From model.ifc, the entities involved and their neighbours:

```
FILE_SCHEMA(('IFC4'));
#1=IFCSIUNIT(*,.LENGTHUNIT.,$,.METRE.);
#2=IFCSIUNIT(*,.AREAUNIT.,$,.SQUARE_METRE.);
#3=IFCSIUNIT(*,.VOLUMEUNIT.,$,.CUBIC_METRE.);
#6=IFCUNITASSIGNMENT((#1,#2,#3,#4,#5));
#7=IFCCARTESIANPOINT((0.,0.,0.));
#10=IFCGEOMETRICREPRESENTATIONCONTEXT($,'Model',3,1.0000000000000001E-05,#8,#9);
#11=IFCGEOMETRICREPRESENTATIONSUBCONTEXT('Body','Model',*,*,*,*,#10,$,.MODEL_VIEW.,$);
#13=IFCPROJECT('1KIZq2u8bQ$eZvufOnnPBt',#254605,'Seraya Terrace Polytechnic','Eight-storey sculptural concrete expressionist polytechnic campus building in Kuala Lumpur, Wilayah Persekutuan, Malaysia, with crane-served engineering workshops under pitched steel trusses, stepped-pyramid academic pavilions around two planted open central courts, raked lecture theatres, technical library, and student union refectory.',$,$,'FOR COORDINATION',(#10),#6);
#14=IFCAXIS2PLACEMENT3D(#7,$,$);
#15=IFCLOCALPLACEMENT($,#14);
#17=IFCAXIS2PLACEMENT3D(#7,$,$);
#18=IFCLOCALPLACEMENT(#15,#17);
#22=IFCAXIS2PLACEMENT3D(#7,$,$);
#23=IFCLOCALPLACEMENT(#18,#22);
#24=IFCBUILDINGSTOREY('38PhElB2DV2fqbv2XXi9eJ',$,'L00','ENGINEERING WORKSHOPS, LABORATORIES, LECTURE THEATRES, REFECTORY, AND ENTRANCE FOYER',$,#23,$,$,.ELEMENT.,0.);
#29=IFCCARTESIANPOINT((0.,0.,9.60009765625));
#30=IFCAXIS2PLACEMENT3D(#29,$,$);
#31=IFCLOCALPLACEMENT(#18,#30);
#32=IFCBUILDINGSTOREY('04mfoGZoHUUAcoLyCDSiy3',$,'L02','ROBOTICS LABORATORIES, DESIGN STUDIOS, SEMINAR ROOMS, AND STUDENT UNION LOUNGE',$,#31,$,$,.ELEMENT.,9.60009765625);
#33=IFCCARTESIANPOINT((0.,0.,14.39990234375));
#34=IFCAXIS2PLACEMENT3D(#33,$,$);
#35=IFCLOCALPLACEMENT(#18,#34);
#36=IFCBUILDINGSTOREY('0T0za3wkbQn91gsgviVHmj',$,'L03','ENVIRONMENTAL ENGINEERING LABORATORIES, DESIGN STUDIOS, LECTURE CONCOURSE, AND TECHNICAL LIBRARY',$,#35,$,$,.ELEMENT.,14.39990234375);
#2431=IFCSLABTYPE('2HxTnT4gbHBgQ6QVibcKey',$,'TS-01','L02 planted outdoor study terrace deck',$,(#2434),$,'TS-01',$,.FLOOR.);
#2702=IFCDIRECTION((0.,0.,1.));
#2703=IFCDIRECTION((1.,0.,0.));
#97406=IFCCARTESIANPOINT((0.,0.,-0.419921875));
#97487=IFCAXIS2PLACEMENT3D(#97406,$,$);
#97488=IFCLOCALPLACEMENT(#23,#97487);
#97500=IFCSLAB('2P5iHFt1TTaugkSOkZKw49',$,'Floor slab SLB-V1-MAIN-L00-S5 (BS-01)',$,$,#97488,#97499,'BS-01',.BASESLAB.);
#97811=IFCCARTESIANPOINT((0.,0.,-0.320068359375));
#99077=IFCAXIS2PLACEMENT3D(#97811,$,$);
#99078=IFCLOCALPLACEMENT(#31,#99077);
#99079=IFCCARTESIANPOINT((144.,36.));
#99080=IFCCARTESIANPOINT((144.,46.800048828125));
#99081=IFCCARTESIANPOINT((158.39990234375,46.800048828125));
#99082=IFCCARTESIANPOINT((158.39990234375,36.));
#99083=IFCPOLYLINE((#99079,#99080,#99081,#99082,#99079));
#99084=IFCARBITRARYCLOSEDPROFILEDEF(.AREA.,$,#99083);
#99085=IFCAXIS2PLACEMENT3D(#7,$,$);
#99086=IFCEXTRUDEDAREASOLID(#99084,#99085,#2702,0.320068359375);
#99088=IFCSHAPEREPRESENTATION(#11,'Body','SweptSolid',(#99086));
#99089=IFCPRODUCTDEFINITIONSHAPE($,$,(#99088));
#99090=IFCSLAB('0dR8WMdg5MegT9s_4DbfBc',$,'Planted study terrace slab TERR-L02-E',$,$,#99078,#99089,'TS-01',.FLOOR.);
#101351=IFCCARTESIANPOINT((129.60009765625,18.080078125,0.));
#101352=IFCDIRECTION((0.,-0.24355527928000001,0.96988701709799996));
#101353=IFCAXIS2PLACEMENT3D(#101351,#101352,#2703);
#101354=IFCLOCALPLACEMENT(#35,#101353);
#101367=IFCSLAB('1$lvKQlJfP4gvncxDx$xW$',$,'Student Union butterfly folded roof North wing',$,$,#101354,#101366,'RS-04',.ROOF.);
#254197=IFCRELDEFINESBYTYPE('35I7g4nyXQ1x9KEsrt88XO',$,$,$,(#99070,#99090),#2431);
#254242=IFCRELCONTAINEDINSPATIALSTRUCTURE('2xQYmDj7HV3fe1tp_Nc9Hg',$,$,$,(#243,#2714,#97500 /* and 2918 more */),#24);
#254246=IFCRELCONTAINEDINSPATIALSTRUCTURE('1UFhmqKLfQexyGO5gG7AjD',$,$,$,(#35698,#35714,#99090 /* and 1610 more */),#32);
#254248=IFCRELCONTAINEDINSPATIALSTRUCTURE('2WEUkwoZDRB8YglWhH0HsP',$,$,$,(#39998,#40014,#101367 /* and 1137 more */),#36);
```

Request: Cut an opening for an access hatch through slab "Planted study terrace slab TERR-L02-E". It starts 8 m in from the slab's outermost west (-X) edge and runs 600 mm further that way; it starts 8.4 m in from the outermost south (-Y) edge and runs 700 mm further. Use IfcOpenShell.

```python
import numpy as np
import ifcopenshell
import ifcopenshell.api.feature
import ifcopenshell.api.geometry
import ifcopenshell.api.root
import ifcopenshell.geom
import ifcopenshell.util.placement
import ifcopenshell.util.representation
import ifcopenshell.util.shape
import ifcopenshell.util.unit

model = ifcopenshell.open("model.ifc")
unit_scale = ifcopenshell.util.unit.calculate_unit_scale(model)
settings = ifcopenshell.geom.settings()


def volume(element):
    """Net volume in cubic metres, openings subtracted."""
    shape = ifcopenshell.geom.create_shape(settings, element)
    return ifcopenshell.util.shape.get_volume(shape.geometry)


slab = model.by_guid("0dR8WMdg5MegT9s_4DbfBc")
before = volume(slab)

# Extent in the slab's own axes, in metres. The edges named are its -X and -Y sides.
slab_shape = ifcopenshell.geom.create_shape(settings, slab)
vertices = ifcopenshell.util.shape.get_vertices(slab_shape.geometry)
x_min, y_min, bottom = vertices.min(axis=0)
top = vertices[:, 2].max()

opening = ifcopenshell.api.root.create_entity(model, ifc_class="IfcOpeningElement", name="Access hatch opening", predefined_type="OPENING")
context = ifcopenshell.util.representation.get_context(model, "Model", "Body", "MODEL_VIEW")
width, depth = 0.6, 0.7
outline = [(0.0, 0.0), (width, 0.0), (width, depth), (0.0, depth), (0.0, 0.0)]
# Overshoot both faces by 50 mm so the cut is clean.
shape = ifcopenshell.api.geometry.add_slab_representation(
    model, context=context, depth=top - bottom + 0.1, polyline=outline
)
ifcopenshell.api.geometry.assign_representation(model, product=opening, representation=shape)

matrix = ifcopenshell.util.placement.get_local_placement(slab.ObjectPlacement)
matrix[:, 3] = matrix @ np.append(np.array([x_min + 8, y_min + 8.4, bottom - 0.05]) / unit_scale, 1.0)
ifcopenshell.api.geometry.edit_object_placement(model, product=opening, matrix=matrix, is_si=False)
ifcopenshell.api.feature.add_feature(model, feature=opening, element=slab)

after = volume(slab)

print(f"slab volume {before:.3f} -> {after:.3f} m3")

model.write("model_rev.ifc")
```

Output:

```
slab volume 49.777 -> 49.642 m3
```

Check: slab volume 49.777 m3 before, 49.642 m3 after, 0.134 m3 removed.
